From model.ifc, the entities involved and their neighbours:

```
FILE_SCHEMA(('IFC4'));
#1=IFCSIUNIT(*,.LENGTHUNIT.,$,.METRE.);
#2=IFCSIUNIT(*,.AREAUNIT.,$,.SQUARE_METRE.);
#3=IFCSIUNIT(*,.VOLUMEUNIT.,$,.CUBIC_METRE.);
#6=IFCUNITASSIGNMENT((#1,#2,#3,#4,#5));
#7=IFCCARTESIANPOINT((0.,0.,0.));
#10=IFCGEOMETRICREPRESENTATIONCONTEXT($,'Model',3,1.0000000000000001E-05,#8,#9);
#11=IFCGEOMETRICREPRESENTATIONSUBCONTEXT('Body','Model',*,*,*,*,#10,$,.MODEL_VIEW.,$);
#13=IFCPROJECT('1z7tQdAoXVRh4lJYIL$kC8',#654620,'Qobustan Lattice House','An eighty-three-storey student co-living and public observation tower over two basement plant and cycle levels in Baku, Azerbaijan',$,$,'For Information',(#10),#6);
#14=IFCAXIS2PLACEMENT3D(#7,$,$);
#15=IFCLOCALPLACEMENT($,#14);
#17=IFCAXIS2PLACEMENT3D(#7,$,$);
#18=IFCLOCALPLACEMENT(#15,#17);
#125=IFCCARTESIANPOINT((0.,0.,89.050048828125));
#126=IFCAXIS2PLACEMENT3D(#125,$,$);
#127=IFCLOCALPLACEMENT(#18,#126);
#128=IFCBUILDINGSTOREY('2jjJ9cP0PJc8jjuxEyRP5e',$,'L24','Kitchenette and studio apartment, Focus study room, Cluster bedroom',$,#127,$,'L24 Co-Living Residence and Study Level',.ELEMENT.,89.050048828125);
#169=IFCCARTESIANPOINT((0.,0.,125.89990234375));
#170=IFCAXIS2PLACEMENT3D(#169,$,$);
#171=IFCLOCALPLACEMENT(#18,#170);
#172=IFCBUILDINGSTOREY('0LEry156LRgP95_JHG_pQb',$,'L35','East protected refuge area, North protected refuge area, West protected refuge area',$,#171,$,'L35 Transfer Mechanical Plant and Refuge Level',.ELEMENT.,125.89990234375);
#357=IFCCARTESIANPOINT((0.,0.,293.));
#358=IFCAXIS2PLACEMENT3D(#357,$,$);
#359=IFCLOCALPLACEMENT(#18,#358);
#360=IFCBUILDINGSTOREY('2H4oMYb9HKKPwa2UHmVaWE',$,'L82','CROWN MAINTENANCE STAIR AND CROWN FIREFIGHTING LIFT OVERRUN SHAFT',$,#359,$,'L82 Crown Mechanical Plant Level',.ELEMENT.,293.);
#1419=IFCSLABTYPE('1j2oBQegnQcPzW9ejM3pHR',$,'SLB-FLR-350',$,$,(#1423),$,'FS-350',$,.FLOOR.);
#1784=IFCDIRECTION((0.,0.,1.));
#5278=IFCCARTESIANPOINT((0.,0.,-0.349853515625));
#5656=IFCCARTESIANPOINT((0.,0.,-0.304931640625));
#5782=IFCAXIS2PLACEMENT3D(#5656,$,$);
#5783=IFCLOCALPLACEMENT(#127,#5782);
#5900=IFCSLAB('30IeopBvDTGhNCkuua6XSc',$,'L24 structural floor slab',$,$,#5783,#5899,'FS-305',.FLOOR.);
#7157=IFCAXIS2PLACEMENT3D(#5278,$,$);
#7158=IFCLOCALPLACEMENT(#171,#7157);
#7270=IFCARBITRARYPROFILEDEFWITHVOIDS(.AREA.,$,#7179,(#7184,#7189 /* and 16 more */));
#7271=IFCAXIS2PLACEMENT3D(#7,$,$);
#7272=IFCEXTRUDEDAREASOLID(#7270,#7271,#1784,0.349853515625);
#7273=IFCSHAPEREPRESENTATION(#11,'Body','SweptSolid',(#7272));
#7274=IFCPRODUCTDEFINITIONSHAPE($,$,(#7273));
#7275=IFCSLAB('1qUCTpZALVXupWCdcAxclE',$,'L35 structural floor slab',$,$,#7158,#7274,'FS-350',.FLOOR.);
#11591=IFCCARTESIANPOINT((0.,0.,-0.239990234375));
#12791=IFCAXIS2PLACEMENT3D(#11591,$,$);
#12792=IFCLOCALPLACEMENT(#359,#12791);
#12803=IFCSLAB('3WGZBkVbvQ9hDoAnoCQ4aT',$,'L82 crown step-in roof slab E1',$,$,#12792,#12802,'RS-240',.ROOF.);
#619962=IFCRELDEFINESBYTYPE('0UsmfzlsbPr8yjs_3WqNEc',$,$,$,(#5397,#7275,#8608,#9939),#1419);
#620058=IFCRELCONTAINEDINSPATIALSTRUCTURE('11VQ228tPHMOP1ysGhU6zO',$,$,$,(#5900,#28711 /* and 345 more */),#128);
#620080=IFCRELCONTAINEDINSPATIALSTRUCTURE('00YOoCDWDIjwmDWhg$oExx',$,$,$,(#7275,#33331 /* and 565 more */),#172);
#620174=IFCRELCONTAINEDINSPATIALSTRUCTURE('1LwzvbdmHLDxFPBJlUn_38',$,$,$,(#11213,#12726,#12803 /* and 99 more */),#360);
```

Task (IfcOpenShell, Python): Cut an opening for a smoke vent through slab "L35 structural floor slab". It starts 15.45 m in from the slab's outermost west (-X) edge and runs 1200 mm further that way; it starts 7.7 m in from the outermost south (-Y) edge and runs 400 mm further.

```python
import numpy as np
import ifcopenshell
import ifcopenshell.api.feature
import ifcopenshell.api.geometry
import ifcopenshell.api.root
import ifcopenshell.geom
import ifcopenshell.util.placement
import ifcopenshell.util.representation
import ifcopenshell.util.shape
import ifcopenshell.util.unit

model = ifcopenshell.open("model.ifc")
unit_scale = ifcopenshell.util.unit.calculate_unit_scale(model)
settings = ifcopenshell.geom.settings()


def volume(element):
    """Net volume in cubic metres, openings subtracted."""
    shape = ifcopenshell.geom.create_shape(settings, element)
    return ifcopenshell.util.shape.get_volume(shape.geometry)


slab = model.by_guid("1qUCTpZALVXupWCdcAxclE")
before = volume(slab)

# Extent in the slab's own axes, in metres. The edges named are its -X and -Y sides.
slab_shape = ifcopenshell.geom.create_shape(settings, slab)
vertices = ifcopenshell.util.shape.get_vertices(slab_shape.geometry)
x_min, y_min, bottom = vertices.min(axis=0)
top = vertices[:, 2].max()

opening = ifcopenshell.api.root.create_entity(model, ifc_class="IfcOpeningElement", name="Smoke vent opening", predefined_type="OPENING")
context = ifcopenshell.util.representation.get_context(model, "Model", "Body", "MODEL_VIEW")
width, depth = 1.2, 0.4
outline = [(0.0, 0.0), (width, 0.0), (width, depth), (0.0, depth), (0.0, 0.0)]
# Overshoot both faces by 50 mm so the cut is clean.
shape = ifcopenshell.api.geometry.add_slab_representation(
    model, context=context, depth=top - bottom + 0.1, polyline=outline
)
ifcopenshell.api.geometry.assign_representation(model, product=opening, representation=shape)

matrix = ifcopenshell.util.placement.get_local_placement(slab.ObjectPlacement)
matrix[:, 3] = matrix @ np.append(np.array([x_min + 15.45, y_min + 7.7, bottom - 0.05]) / unit_scale, 1.0)
ifcopenshell.api.geometry.edit_object_placement(model, product=opening, matrix=matrix, is_si=False)
ifcopenshell.api.feature.add_feature(model, feature=opening, element=slab)

after = volume(slab)

print(f"slab volume {before:.3f} -> {after:.3f} m3")

model.write("model_updated.ifc")
```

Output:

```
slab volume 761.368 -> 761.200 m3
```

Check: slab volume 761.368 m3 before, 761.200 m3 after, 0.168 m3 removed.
